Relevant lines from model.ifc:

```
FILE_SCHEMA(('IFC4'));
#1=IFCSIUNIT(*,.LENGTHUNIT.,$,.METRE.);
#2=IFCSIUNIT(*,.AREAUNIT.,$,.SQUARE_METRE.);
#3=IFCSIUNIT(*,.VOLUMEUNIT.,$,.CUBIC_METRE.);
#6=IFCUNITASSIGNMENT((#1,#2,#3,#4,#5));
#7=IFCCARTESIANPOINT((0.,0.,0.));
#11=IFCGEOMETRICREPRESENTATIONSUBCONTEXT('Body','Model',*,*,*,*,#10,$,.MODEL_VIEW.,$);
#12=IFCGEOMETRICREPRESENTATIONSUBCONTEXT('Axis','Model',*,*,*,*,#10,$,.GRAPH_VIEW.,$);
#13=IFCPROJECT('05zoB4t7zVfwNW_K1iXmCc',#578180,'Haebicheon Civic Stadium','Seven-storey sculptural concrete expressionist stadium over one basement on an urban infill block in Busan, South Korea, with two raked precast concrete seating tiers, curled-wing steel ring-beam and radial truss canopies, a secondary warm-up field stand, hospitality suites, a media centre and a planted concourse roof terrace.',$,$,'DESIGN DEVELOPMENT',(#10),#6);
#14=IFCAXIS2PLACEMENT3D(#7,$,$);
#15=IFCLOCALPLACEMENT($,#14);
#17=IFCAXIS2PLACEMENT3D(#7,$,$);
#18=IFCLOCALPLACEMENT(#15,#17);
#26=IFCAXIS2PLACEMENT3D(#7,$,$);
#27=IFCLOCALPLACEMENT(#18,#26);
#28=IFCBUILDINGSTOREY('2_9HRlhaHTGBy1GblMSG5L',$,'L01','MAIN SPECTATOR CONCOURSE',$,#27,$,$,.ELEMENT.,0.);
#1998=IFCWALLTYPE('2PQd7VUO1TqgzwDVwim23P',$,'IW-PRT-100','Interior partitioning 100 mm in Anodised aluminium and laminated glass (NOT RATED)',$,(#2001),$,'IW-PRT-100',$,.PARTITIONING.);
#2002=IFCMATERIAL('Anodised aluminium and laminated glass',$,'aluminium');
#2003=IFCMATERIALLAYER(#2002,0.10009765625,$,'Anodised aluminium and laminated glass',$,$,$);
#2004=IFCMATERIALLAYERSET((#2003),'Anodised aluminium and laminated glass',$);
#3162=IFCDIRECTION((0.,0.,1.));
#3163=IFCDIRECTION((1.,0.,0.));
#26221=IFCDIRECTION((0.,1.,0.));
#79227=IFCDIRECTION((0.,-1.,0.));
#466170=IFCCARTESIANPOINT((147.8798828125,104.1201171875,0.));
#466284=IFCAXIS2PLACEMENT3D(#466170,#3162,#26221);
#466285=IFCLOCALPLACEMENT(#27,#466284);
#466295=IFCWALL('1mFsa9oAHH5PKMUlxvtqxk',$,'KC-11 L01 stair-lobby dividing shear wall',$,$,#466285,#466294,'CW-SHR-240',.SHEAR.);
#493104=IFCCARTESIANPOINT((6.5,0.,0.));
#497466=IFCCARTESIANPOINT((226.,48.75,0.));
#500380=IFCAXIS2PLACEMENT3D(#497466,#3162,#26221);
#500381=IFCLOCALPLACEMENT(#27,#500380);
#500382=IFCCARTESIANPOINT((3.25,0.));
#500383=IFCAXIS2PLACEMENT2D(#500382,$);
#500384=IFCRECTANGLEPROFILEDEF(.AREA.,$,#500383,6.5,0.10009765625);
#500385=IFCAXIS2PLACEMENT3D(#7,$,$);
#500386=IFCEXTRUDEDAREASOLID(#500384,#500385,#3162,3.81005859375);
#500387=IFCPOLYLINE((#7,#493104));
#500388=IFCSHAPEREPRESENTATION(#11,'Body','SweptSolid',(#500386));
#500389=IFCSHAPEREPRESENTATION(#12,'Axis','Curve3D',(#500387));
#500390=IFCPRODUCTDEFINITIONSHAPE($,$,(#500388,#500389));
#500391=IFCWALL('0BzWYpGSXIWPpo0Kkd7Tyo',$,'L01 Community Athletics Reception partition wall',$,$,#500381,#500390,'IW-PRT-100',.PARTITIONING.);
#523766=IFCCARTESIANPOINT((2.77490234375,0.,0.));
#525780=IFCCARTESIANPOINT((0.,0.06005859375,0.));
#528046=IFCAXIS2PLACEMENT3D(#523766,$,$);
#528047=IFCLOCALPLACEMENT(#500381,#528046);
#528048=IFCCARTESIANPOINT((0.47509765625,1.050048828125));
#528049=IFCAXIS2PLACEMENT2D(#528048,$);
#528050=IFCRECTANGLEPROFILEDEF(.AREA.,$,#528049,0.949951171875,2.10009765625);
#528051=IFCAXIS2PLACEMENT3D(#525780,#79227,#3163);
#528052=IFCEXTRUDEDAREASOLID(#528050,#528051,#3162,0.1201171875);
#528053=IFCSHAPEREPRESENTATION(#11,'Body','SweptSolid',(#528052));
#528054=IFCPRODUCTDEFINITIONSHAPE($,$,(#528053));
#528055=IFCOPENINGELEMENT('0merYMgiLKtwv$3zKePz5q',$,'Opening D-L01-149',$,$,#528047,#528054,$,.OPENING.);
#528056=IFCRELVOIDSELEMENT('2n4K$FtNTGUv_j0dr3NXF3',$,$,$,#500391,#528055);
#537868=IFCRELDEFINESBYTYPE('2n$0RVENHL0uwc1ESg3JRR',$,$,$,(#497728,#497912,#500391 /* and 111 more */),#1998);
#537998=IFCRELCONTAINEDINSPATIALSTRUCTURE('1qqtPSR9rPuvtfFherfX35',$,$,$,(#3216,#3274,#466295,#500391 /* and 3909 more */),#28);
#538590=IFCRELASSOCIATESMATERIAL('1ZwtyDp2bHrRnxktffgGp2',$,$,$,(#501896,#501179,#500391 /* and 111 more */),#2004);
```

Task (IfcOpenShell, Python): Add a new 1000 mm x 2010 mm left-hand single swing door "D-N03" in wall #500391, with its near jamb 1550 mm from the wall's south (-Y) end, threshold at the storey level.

```python
import numpy as np
import ifcopenshell
import ifcopenshell.api.feature
import ifcopenshell.api.geometry
import ifcopenshell.api.root
import ifcopenshell.api.spatial
import ifcopenshell.geom
import ifcopenshell.util.element
import ifcopenshell.util.placement
import ifcopenshell.util.representation
import ifcopenshell.util.shape
import ifcopenshell.util.unit

model = ifcopenshell.open("model.ifc")
unit_scale = ifcopenshell.util.unit.calculate_unit_scale(model)
settings = ifcopenshell.geom.settings()


def volume(element):
    """Net volume in cubic metres, openings subtracted."""
    shape = ifcopenshell.geom.create_shape(settings, element)
    return ifcopenshell.util.shape.get_volume(shape.geometry)


wall = model.by_id(500391)
storey = ifcopenshell.util.element.get_container(wall, ifc_class="IfcBuildingStorey")
context = ifcopenshell.util.representation.get_context(model, "Model", "Body", "MODEL_VIEW")
before = volume(wall)

width, height, from_end, sill = 1, 2.01, 1.55, 0.0  # metres

# The wall runs along its own X axis, and the end named is its -X end.
wall_shape = ifcopenshell.geom.create_shape(settings, wall)
x, y, z = ifcopenshell.util.shape.get_vertices(wall_shape.geometry).T
start = x.min() + from_end
face, thickness = float(y.min()), float(y.max() - y.min())
wall_matrix = ifcopenshell.util.placement.get_local_placement(wall.ObjectPlacement)
level = ifcopenshell.util.placement.get_local_placement(storey.ObjectPlacement)[2, 3]


def in_wall(x, y):
    """Placement at x, y metres in the wall's axes, at sill height."""
    matrix = wall_matrix.copy()
    matrix[:, 3] = wall_matrix @ np.array([x / unit_scale, y / unit_scale, 0.0, 1.0])
    matrix[2, 3] = level + sill / unit_scale
    return matrix


# Opening: a box that overshoots both wall faces by 50 mm.
opening = ifcopenshell.api.root.create_entity(model, ifc_class="IfcOpeningElement", predefined_type="OPENING")
box = ifcopenshell.api.geometry.add_wall_representation(
    model, context=context, length=width, height=height, thickness=thickness + 0.1
)
ifcopenshell.api.geometry.assign_representation(model, product=opening, representation=box)
ifcopenshell.api.geometry.edit_object_placement(model, product=opening, matrix=in_wall(start, face - 0.05), is_si=False)
ifcopenshell.api.feature.add_feature(model, feature=opening, element=wall)

door = ifcopenshell.api.root.create_entity(model, ifc_class="IfcDoor", name="D-N03", predefined_type="DOOR")
door.OverallWidth, door.OverallHeight = width / unit_scale, height / unit_scale
door.OperationType = "SINGLE_SWING_LEFT"
body = ifcopenshell.api.geometry.add_door_representation(
    model,
    context=context,
    overall_width=door.OverallWidth,
    overall_height=door.OverallHeight,
    operation_type="SINGLE_SWING_LEFT",
    lining_properties={"LiningDepth": thickness / unit_scale, "ThresholdDepth": thickness / unit_scale},
)
ifcopenshell.api.geometry.assign_representation(model, product=door, representation=body)
ifcopenshell.api.spatial.assign_container(model, products=[door], relating_structure=storey)
ifcopenshell.api.feature.add_filling(model, opening=opening, element=door)

# The lining spans the wall, so the door starts at the wall face.
ifcopenshell.api.geometry.edit_object_placement(model, product=door, matrix=in_wall(start, face), is_si=False)

after = volume(wall)

print(f"wall volume {before:.3f} -> {after:.3f} m3")

model.write("model_edited.ifc")
```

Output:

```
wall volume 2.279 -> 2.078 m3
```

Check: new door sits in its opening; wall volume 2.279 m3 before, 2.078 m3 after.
